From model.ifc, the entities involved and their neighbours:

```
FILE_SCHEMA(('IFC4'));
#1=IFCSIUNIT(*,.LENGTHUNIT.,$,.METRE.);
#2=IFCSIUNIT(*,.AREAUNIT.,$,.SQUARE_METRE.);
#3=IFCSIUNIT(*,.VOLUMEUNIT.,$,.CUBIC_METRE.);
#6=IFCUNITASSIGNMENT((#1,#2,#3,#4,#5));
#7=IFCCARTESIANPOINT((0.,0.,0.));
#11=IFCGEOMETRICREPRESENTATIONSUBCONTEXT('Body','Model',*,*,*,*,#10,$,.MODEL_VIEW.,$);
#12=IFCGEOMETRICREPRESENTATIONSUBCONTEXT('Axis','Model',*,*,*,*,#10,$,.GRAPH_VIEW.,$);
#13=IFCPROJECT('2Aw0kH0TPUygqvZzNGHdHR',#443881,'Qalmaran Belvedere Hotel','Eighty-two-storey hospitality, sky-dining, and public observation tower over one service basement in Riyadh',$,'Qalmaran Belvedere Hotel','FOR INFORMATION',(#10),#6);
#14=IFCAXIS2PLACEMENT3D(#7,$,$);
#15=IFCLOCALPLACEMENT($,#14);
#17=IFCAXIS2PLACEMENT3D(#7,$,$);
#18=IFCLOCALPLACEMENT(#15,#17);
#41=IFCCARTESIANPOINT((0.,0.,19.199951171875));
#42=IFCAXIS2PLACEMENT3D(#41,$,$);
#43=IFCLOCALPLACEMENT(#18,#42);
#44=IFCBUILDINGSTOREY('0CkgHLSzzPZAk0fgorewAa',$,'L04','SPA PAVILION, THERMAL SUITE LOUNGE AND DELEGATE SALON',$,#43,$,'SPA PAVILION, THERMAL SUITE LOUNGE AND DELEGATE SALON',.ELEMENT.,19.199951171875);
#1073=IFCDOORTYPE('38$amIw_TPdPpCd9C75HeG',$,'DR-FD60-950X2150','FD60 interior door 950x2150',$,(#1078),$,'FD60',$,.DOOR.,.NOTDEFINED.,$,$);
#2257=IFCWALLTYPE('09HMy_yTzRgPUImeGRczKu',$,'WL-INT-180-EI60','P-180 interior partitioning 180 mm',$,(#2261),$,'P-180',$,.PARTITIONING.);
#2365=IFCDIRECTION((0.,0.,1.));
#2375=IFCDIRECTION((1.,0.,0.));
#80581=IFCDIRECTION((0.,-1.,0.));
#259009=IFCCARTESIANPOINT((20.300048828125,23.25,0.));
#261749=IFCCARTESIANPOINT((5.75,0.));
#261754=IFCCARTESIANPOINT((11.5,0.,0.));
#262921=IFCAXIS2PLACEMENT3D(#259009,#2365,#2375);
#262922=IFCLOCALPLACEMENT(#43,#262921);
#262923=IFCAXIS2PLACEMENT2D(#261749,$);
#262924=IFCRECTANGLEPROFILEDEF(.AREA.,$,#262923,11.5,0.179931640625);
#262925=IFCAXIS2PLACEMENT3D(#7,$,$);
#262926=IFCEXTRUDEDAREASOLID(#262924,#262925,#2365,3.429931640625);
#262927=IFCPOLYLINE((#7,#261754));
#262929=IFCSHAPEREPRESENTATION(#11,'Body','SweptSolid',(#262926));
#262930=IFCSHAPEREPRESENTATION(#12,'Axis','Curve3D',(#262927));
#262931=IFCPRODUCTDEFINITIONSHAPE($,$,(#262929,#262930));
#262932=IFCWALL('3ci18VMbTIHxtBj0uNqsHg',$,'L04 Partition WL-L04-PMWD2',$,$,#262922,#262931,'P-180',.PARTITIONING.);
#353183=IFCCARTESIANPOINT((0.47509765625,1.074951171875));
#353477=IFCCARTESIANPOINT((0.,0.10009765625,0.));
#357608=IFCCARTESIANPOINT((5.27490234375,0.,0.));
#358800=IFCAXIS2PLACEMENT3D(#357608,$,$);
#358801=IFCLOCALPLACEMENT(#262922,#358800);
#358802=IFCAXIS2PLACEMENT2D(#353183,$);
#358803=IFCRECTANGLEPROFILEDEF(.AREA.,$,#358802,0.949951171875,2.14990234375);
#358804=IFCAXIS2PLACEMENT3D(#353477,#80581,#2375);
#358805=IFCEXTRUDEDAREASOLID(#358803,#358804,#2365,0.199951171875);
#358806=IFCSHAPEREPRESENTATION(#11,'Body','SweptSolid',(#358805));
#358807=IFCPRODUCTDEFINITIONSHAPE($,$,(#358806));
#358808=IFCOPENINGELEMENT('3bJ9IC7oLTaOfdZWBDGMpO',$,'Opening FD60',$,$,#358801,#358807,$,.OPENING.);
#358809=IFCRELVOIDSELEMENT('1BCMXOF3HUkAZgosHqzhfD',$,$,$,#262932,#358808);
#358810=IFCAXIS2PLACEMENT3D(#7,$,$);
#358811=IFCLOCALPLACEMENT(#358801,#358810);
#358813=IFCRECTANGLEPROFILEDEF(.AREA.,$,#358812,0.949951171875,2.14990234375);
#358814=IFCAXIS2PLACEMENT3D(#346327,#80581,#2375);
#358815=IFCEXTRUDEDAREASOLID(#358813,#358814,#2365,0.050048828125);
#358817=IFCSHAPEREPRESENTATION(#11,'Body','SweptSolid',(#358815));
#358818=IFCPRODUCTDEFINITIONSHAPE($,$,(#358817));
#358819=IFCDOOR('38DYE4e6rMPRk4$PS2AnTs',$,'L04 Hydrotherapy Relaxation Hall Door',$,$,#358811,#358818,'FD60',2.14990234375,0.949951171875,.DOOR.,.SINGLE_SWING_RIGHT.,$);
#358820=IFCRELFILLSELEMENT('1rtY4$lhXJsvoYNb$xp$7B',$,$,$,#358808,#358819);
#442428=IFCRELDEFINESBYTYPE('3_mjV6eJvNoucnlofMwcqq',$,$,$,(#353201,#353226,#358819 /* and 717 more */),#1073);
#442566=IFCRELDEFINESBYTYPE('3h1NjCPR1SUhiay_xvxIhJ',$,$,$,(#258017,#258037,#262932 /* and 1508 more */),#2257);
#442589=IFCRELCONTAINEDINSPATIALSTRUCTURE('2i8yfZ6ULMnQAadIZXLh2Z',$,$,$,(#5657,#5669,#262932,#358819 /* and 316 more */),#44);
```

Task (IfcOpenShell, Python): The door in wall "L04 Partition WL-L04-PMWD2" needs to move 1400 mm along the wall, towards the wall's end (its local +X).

```python
import ifcopenshell
import ifcopenshell.api.geometry
import ifcopenshell.util.placement
import ifcopenshell.util.unit

model = ifcopenshell.open("model.ifc")
unit_scale = ifcopenshell.util.unit.calculate_unit_scale(model)

door = model.by_id(358819)
opening = door.FillsVoids[0].RelatingOpeningElement
wall = opening.VoidsElements[0].RelatingBuildingElement

wall_matrix = ifcopenshell.util.placement.get_local_placement(wall.ObjectPlacement)
shift = wall_matrix[:3, 0] * 1.4 / unit_scale
before = ifcopenshell.util.placement.get_local_placement(door.ObjectPlacement)[:3, 3].copy()

# The door is placed relative to its opening, so it follows when the opening moves.
matrix = ifcopenshell.util.placement.get_local_placement(opening.ObjectPlacement)
matrix[:3, 3] += shift
ifcopenshell.api.geometry.edit_object_placement(
    model, product=opening, matrix=matrix, is_si=False, should_transform_children=True
)

after = ifcopenshell.util.placement.get_local_placement(door.ObjectPlacement)[:3, 3]
print("door moved by", (after - before).round(3) + 0.0)

model.write("model_updated.ifc")
```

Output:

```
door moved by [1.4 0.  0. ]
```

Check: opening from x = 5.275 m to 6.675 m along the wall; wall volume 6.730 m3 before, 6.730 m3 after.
